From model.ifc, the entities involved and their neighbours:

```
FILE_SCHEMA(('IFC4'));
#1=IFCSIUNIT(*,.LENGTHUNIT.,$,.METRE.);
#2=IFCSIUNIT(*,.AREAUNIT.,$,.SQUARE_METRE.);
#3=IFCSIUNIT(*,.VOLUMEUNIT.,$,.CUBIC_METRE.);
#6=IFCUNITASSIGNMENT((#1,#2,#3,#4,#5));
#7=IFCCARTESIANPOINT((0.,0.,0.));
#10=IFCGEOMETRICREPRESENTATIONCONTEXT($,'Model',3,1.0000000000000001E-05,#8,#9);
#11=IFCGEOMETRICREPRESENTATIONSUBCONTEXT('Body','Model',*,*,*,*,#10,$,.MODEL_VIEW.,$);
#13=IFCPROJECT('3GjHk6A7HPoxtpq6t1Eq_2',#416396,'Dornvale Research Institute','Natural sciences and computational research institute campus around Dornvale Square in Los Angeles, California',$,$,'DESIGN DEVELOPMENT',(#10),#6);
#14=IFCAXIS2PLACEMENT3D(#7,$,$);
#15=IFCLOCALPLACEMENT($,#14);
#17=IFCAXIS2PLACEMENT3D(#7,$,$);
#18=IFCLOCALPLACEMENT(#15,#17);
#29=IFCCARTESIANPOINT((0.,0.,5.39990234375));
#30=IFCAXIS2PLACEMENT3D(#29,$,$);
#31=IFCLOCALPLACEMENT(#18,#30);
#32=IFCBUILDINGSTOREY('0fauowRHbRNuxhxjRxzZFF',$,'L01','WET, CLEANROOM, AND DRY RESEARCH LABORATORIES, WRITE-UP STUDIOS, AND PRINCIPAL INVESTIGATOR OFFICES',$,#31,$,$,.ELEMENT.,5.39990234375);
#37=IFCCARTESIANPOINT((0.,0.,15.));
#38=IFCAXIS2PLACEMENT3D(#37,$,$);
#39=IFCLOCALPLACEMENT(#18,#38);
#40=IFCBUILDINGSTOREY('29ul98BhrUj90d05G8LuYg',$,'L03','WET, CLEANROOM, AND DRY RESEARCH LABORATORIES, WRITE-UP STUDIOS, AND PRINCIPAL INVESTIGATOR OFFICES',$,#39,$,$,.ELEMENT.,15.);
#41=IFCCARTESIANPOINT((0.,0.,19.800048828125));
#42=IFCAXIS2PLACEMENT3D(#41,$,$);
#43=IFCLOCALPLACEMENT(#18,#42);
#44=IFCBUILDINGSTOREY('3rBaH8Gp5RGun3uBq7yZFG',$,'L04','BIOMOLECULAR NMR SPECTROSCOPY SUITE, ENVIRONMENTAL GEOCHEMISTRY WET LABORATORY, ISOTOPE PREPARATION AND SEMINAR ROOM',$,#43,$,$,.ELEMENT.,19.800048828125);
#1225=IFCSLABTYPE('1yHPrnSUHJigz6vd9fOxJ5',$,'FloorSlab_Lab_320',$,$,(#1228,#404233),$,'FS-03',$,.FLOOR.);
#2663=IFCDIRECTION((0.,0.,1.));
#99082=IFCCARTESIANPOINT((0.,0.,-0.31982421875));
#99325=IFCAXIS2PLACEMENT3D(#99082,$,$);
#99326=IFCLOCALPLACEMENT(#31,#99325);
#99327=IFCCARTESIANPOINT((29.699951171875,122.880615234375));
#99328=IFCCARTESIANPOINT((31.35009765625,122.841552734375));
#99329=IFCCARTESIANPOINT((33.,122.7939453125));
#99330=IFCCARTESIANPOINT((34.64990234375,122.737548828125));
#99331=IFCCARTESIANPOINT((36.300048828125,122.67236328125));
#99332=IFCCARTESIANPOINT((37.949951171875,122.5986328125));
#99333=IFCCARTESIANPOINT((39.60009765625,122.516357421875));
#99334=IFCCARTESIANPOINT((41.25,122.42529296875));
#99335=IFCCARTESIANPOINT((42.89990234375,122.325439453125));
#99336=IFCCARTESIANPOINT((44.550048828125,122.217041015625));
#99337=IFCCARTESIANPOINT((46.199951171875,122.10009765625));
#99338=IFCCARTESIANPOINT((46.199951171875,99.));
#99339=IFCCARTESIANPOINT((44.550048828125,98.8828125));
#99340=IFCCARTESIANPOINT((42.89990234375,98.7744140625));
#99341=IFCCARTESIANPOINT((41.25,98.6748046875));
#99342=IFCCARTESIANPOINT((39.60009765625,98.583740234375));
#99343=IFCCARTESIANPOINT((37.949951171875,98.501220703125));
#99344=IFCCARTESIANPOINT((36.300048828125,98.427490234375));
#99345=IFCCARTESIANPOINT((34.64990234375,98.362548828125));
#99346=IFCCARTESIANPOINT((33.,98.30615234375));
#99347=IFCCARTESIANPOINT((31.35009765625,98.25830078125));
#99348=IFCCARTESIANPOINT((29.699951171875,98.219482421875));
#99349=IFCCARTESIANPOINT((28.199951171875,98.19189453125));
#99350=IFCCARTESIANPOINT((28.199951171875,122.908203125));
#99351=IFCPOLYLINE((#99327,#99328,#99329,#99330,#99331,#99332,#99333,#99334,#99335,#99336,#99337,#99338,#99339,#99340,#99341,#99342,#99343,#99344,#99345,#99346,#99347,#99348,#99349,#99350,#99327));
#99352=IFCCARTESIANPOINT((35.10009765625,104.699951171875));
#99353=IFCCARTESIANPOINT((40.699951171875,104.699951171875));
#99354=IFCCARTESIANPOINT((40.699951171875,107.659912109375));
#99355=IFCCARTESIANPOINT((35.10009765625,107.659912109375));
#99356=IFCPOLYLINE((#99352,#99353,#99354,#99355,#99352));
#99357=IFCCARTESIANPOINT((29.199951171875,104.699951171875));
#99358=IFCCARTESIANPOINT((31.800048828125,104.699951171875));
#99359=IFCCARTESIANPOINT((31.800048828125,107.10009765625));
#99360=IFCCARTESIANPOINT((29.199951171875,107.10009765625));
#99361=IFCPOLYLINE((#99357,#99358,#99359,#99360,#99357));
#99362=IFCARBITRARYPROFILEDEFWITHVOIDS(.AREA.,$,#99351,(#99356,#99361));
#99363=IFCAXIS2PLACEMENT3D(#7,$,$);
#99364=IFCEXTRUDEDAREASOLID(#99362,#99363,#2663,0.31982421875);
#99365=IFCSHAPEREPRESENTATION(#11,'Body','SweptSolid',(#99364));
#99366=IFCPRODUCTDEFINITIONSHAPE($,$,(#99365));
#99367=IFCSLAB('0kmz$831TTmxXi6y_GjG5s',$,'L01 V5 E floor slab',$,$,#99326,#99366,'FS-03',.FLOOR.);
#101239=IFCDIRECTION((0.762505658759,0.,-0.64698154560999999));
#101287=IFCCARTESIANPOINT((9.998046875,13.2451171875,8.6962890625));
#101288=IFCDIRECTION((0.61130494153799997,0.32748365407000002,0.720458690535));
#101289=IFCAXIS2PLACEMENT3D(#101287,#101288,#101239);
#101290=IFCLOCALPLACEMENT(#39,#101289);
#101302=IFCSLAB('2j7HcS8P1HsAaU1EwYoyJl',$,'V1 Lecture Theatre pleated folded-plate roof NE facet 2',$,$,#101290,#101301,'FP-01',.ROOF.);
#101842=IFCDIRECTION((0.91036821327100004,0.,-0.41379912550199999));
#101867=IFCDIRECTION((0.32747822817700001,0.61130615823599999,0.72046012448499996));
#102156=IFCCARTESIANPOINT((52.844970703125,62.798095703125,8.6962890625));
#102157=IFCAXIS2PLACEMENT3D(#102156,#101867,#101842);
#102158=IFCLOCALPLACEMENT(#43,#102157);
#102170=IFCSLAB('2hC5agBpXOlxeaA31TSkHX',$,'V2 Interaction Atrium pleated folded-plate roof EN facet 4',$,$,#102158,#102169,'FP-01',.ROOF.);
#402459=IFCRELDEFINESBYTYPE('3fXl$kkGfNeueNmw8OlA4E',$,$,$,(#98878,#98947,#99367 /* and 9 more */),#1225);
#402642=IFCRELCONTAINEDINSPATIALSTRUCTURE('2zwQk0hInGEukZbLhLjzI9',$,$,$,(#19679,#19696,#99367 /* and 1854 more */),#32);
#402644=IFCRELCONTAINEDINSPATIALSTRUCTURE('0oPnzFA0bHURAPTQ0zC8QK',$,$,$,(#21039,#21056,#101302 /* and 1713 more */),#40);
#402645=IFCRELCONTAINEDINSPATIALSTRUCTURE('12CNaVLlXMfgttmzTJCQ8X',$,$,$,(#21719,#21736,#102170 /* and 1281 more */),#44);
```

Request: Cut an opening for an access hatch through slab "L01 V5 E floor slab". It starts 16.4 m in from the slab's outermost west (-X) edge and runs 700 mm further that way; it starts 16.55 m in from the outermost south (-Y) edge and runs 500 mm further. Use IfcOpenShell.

```python
import numpy as np
import ifcopenshell
import ifcopenshell.api.feature
import ifcopenshell.api.geometry
import ifcopenshell.api.root
import ifcopenshell.geom
import ifcopenshell.util.placement
import ifcopenshell.util.representation
import ifcopenshell.util.shape
import ifcopenshell.util.unit

model = ifcopenshell.open("model.ifc")
unit_scale = ifcopenshell.util.unit.calculate_unit_scale(model)
settings = ifcopenshell.geom.settings()


def volume(element):
    """Net volume in cubic metres, openings subtracted."""
    shape = ifcopenshell.geom.create_shape(settings, element)
    return ifcopenshell.util.shape.get_volume(shape.geometry)


slab = model.by_id(99367)
before = volume(slab)

# Extent in the slab's own axes, in metres. The edges named are its -X and -Y sides.
slab_shape = ifcopenshell.geom.create_shape(settings, slab)
vertices = ifcopenshell.util.shape.get_vertices(slab_shape.geometry)
x_min, y_min, bottom = vertices.min(axis=0)
top = vertices[:, 2].max()

opening = ifcopenshell.api.root.create_entity(model, ifc_class="IfcOpeningElement", name="Access hatch opening", predefined_type="OPENING")
context = ifcopenshell.util.representation.get_context(model, "Model", "Body", "MODEL_VIEW")
width, depth = 0.7, 0.5
outline = [(0.0, 0.0), (width, 0.0), (width, depth), (0.0, depth), (0.0, 0.0)]
# Overshoot both faces by 50 mm so the cut is clean.
shape = ifcopenshell.api.geometry.add_slab_representation(
    model, context=context, depth=top - bottom + 0.1, polyline=outline
)
ifcopenshell.api.geometry.assign_representation(model, product=opening, representation=shape)

matrix = ifcopenshell.util.placement.get_local_placement(slab.ObjectPlacement)
matrix[:, 3] = matrix @ np.append(np.array([x_min + 16.4, y_min + 16.55, bottom - 0.05]) / unit_scale, 1.0)
ifcopenshell.api.geometry.edit_object_placement(model, product=opening, matrix=matrix, is_si=False)
ifcopenshell.api.feature.add_feature(model, feature=opening, element=slab)

after = volume(slab)

print(f"slab volume {before:.3f} -> {after:.3f} m3")

model.write("model_v2.ifc")
```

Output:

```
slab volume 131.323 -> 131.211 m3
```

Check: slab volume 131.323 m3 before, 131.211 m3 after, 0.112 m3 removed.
